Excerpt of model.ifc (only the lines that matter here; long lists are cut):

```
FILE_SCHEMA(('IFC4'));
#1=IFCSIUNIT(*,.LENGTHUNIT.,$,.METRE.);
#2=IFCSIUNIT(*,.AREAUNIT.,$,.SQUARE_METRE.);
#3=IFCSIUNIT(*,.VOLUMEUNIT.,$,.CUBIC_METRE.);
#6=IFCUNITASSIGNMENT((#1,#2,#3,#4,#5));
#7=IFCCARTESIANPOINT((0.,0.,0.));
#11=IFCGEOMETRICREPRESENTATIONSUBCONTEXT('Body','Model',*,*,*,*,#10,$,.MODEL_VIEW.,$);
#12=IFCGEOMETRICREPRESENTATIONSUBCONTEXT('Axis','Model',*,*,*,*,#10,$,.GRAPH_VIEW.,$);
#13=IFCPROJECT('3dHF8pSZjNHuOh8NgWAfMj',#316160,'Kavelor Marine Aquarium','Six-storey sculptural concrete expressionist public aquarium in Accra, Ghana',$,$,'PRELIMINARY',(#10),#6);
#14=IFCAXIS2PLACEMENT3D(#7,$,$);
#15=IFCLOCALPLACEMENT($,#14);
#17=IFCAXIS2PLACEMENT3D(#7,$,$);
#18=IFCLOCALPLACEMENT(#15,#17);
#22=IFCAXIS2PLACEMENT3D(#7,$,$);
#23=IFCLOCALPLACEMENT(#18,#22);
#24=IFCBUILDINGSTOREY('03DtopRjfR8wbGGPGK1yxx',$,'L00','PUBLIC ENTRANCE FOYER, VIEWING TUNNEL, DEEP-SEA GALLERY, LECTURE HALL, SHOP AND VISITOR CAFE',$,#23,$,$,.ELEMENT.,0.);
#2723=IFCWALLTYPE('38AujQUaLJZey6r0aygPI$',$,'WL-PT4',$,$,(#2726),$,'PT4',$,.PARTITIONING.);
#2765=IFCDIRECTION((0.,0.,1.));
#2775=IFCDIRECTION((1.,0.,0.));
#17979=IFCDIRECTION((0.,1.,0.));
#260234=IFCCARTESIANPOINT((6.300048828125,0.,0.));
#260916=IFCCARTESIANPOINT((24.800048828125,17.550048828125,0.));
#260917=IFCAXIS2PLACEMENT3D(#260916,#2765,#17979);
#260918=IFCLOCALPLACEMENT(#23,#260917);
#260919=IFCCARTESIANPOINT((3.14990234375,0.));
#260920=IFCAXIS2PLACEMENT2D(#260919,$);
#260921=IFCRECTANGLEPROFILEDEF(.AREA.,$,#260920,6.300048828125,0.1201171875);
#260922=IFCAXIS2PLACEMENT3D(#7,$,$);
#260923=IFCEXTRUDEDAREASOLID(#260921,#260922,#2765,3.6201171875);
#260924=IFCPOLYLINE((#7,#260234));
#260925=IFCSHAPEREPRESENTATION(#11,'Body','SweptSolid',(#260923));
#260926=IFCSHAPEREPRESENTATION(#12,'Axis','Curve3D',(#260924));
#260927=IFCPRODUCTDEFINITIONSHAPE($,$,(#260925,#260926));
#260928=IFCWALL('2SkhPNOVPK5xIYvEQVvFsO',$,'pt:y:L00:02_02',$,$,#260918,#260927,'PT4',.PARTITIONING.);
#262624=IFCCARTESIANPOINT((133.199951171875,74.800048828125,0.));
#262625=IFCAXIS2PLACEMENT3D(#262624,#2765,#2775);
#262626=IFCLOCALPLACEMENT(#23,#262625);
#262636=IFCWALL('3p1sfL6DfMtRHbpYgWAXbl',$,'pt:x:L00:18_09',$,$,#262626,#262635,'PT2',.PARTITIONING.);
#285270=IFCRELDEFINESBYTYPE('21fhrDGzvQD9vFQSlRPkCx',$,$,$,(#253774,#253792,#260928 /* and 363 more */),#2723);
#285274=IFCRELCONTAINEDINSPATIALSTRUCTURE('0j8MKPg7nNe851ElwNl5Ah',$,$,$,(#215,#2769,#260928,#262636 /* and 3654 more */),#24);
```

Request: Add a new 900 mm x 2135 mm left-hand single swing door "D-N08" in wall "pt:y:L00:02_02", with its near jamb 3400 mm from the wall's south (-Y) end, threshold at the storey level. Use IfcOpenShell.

```python
import numpy as np
import ifcopenshell
import ifcopenshell.api.feature
import ifcopenshell.api.geometry
import ifcopenshell.api.root
import ifcopenshell.api.spatial
import ifcopenshell.geom
import ifcopenshell.util.element
import ifcopenshell.util.placement
import ifcopenshell.util.representation
import ifcopenshell.util.shape
import ifcopenshell.util.unit

model = ifcopenshell.open("model.ifc")
unit_scale = ifcopenshell.util.unit.calculate_unit_scale(model)
settings = ifcopenshell.geom.settings()


def volume(element):
    """Net volume in cubic metres, openings subtracted."""
    shape = ifcopenshell.geom.create_shape(settings, element)
    return ifcopenshell.util.shape.get_volume(shape.geometry)


wall = model.by_guid("2SkhPNOVPK5xIYvEQVvFsO")
storey = ifcopenshell.util.element.get_container(wall, ifc_class="IfcBuildingStorey")
context = ifcopenshell.util.representation.get_context(model, "Model", "Body", "MODEL_VIEW")
before = volume(wall)

width, height, from_end, sill = 0.9, 2.135, 3.4, 0.0  # metres

# The wall runs along its own X axis, and the end named is its -X end.
wall_shape = ifcopenshell.geom.create_shape(settings, wall)
x, y, z = ifcopenshell.util.shape.get_vertices(wall_shape.geometry).T
start = x.min() + from_end
face, thickness = float(y.min()), float(y.max() - y.min())
wall_matrix = ifcopenshell.util.placement.get_local_placement(wall.ObjectPlacement)
level = ifcopenshell.util.placement.get_local_placement(storey.ObjectPlacement)[2, 3]


def in_wall(x, y):
    """Placement at x, y metres in the wall's axes, at sill height."""
    matrix = wall_matrix.copy()
    matrix[:, 3] = wall_matrix @ np.array([x / unit_scale, y / unit_scale, 0.0, 1.0])
    matrix[2, 3] = level + sill / unit_scale
    return matrix


# Opening: a box that overshoots both wall faces by 50 mm.
opening = ifcopenshell.api.root.create_entity(model, ifc_class="IfcOpeningElement", predefined_type="OPENING")
box = ifcopenshell.api.geometry.add_wall_representation(
    model, context=context, length=width, height=height, thickness=thickness + 0.1
)
ifcopenshell.api.geometry.assign_representation(model, product=opening, representation=box)
ifcopenshell.api.geometry.edit_object_placement(model, product=opening, matrix=in_wall(start, face - 0.05), is_si=False)
ifcopenshell.api.feature.add_feature(model, feature=opening, element=wall)

door = ifcopenshell.api.root.create_entity(model, ifc_class="IfcDoor", name="D-N08", predefined_type="DOOR")
door.OverallWidth, door.OverallHeight = width / unit_scale, height / unit_scale
door.OperationType = "SINGLE_SWING_LEFT"
body = ifcopenshell.api.geometry.add_door_representation(
    model,
    context=context,
    overall_width=door.OverallWidth,
    overall_height=door.OverallHeight,
    operation_type="SINGLE_SWING_LEFT",
    lining_properties={"LiningDepth": thickness / unit_scale, "ThresholdDepth": thickness / unit_scale},
)
ifcopenshell.api.geometry.assign_representation(model, product=door, representation=body)
ifcopenshell.api.spatial.assign_container(model, products=[door], relating_structure=storey)
ifcopenshell.api.feature.add_filling(model, opening=opening, element=door)

# The lining spans the wall, so the door starts at the wall face.
ifcopenshell.api.geometry.edit_object_placement(model, product=door, matrix=in_wall(start, face), is_si=False)

after = volume(wall)

print(f"wall volume {before:.3f} -> {after:.3f} m3")

model.write("model_updated.ifc")
```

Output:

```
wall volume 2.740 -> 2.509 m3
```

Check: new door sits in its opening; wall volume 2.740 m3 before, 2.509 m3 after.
